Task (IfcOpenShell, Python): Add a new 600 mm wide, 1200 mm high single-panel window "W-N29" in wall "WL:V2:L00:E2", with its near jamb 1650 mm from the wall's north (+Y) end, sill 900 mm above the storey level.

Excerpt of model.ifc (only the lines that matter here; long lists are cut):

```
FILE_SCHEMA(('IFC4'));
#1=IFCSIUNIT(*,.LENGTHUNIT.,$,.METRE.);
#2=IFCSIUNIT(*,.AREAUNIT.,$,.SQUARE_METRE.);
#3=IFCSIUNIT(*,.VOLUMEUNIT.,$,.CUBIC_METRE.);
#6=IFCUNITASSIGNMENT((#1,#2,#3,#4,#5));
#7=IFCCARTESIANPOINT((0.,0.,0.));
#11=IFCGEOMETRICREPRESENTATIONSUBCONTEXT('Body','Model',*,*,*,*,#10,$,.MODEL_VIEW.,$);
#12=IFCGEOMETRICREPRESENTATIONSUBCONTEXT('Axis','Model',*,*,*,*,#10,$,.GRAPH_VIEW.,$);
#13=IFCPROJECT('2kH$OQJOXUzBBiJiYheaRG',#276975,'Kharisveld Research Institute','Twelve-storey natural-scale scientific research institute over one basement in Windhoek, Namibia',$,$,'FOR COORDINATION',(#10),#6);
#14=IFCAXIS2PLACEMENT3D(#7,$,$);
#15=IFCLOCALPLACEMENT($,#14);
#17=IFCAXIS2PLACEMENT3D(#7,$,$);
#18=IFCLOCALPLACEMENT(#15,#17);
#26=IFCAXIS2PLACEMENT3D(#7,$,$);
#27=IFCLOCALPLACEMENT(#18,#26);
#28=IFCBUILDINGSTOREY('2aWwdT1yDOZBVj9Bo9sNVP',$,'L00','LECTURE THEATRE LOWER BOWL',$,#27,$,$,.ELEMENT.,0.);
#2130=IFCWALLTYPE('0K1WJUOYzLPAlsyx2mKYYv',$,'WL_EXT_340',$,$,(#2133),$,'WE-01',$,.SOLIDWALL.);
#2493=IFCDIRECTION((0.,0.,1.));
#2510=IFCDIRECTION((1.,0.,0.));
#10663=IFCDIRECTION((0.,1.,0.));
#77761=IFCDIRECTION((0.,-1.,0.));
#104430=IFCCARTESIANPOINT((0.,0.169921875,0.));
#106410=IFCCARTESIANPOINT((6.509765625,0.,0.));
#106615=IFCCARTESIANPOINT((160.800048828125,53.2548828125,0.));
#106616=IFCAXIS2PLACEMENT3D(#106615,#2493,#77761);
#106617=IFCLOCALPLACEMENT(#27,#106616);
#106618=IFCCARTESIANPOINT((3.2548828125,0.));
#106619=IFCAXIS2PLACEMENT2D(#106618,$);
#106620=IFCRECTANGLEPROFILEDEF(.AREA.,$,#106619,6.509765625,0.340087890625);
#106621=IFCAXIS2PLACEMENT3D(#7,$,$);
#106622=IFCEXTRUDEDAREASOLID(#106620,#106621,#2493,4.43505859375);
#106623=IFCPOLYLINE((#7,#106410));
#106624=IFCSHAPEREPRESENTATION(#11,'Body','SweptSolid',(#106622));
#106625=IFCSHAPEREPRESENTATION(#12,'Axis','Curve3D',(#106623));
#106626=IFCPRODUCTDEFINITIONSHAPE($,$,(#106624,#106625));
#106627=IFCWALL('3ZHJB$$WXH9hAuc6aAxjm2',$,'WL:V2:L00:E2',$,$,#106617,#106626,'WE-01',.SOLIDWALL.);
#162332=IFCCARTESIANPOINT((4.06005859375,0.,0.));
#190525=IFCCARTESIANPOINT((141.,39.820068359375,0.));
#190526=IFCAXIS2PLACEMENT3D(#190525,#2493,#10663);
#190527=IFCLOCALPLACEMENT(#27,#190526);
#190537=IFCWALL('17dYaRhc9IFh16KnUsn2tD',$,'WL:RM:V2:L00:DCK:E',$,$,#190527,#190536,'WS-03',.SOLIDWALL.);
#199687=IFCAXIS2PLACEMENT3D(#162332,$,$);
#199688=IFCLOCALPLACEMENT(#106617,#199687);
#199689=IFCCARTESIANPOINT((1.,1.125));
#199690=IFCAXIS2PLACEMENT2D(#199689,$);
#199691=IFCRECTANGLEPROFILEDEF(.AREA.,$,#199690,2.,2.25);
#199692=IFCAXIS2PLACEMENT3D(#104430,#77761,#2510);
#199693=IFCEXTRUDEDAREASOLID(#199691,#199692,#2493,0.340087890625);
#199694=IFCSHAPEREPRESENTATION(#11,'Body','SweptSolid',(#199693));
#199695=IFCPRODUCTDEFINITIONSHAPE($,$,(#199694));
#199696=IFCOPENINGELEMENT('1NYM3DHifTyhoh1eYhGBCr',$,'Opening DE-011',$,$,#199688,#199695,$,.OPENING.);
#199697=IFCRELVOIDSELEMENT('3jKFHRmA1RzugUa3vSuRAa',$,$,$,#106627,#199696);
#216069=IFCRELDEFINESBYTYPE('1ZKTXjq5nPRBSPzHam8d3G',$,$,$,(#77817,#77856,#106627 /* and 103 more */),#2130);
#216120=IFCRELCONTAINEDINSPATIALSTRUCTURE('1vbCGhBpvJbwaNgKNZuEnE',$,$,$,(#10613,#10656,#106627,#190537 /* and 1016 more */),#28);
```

```python
import numpy as np
import ifcopenshell
import ifcopenshell.api.feature
import ifcopenshell.api.geometry
import ifcopenshell.api.root
import ifcopenshell.api.spatial
import ifcopenshell.geom
import ifcopenshell.util.element
import ifcopenshell.util.placement
import ifcopenshell.util.representation
import ifcopenshell.util.shape
import ifcopenshell.util.unit

model = ifcopenshell.open("model.ifc")
unit_scale = ifcopenshell.util.unit.calculate_unit_scale(model)
settings = ifcopenshell.geom.settings()


def volume(element):
    """Net volume in cubic metres, openings subtracted."""
    shape = ifcopenshell.geom.create_shape(settings, element)
    return ifcopenshell.util.shape.get_volume(shape.geometry)


wall = model.by_guid("3ZHJB$$WXH9hAuc6aAxjm2")
storey = ifcopenshell.util.element.get_container(wall, ifc_class="IfcBuildingStorey")
context = ifcopenshell.util.representation.get_context(model, "Model", "Body", "MODEL_VIEW")
before = volume(wall)

width, height, from_end, sill = 0.6, 1.2, 1.65, 0.9  # metres

# The wall runs along its own X axis, and the end named is its -X end.
wall_shape = ifcopenshell.geom.create_shape(settings, wall)
x, y, z = ifcopenshell.util.shape.get_vertices(wall_shape.geometry).T
start = x.min() + from_end
face, thickness = float(y.min()), float(y.max() - y.min())
wall_matrix = ifcopenshell.util.placement.get_local_placement(wall.ObjectPlacement)
level = ifcopenshell.util.placement.get_local_placement(storey.ObjectPlacement)[2, 3]


def in_wall(x, y):
    """Placement at x, y metres in the wall's axes, at sill height."""
    matrix = wall_matrix.copy()
    matrix[:, 3] = wall_matrix @ np.array([x / unit_scale, y / unit_scale, 0.0, 1.0])
    matrix[2, 3] = level + sill / unit_scale
    return matrix


# Opening: a box that overshoots both wall faces by 50 mm.
opening = ifcopenshell.api.root.create_entity(model, ifc_class="IfcOpeningElement", predefined_type="OPENING")
box = ifcopenshell.api.geometry.add_wall_representation(
    model, context=context, length=width, height=height, thickness=thickness + 0.1
)
ifcopenshell.api.geometry.assign_representation(model, product=opening, representation=box)
ifcopenshell.api.geometry.edit_object_placement(model, product=opening, matrix=in_wall(start, face - 0.05), is_si=False)
ifcopenshell.api.feature.add_feature(model, feature=opening, element=wall)

window = ifcopenshell.api.root.create_entity(model, ifc_class="IfcWindow", name="W-N29", predefined_type="WINDOW")
window.OverallWidth, window.OverallHeight = width / unit_scale, height / unit_scale
window.PartitioningType = "SINGLE_PANEL"
body = ifcopenshell.api.geometry.add_window_representation(
    model,
    context=context,
    overall_width=window.OverallWidth,
    overall_height=window.OverallHeight,
    partition_type="SINGLE_PANEL",
)
ifcopenshell.api.geometry.assign_representation(model, product=window, representation=body)
ifcopenshell.api.spatial.assign_container(model, products=[window], relating_structure=storey)
ifcopenshell.api.feature.add_filling(model, opening=opening, element=window)

# Centre the window in the wall's thickness.
ifcopenshell.api.geometry.edit_object_placement(model, product=window, matrix=in_wall(start, face), is_si=False)
window_shape = ifcopenshell.geom.create_shape(settings, window)
depth = ifcopenshell.util.shape.get_vertices(window_shape.geometry)[:, 1]
offset = face + thickness / 2 - (depth.min() + depth.max()) / 2
ifcopenshell.api.geometry.edit_object_placement(model, product=window, matrix=in_wall(start, offset), is_si=False)

after = volume(wall)

print(f"wall volume {before:.3f} -> {after:.3f} m3")

model.write("model_v2.ifc")
```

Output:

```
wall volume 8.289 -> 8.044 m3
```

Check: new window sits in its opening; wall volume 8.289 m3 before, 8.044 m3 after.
